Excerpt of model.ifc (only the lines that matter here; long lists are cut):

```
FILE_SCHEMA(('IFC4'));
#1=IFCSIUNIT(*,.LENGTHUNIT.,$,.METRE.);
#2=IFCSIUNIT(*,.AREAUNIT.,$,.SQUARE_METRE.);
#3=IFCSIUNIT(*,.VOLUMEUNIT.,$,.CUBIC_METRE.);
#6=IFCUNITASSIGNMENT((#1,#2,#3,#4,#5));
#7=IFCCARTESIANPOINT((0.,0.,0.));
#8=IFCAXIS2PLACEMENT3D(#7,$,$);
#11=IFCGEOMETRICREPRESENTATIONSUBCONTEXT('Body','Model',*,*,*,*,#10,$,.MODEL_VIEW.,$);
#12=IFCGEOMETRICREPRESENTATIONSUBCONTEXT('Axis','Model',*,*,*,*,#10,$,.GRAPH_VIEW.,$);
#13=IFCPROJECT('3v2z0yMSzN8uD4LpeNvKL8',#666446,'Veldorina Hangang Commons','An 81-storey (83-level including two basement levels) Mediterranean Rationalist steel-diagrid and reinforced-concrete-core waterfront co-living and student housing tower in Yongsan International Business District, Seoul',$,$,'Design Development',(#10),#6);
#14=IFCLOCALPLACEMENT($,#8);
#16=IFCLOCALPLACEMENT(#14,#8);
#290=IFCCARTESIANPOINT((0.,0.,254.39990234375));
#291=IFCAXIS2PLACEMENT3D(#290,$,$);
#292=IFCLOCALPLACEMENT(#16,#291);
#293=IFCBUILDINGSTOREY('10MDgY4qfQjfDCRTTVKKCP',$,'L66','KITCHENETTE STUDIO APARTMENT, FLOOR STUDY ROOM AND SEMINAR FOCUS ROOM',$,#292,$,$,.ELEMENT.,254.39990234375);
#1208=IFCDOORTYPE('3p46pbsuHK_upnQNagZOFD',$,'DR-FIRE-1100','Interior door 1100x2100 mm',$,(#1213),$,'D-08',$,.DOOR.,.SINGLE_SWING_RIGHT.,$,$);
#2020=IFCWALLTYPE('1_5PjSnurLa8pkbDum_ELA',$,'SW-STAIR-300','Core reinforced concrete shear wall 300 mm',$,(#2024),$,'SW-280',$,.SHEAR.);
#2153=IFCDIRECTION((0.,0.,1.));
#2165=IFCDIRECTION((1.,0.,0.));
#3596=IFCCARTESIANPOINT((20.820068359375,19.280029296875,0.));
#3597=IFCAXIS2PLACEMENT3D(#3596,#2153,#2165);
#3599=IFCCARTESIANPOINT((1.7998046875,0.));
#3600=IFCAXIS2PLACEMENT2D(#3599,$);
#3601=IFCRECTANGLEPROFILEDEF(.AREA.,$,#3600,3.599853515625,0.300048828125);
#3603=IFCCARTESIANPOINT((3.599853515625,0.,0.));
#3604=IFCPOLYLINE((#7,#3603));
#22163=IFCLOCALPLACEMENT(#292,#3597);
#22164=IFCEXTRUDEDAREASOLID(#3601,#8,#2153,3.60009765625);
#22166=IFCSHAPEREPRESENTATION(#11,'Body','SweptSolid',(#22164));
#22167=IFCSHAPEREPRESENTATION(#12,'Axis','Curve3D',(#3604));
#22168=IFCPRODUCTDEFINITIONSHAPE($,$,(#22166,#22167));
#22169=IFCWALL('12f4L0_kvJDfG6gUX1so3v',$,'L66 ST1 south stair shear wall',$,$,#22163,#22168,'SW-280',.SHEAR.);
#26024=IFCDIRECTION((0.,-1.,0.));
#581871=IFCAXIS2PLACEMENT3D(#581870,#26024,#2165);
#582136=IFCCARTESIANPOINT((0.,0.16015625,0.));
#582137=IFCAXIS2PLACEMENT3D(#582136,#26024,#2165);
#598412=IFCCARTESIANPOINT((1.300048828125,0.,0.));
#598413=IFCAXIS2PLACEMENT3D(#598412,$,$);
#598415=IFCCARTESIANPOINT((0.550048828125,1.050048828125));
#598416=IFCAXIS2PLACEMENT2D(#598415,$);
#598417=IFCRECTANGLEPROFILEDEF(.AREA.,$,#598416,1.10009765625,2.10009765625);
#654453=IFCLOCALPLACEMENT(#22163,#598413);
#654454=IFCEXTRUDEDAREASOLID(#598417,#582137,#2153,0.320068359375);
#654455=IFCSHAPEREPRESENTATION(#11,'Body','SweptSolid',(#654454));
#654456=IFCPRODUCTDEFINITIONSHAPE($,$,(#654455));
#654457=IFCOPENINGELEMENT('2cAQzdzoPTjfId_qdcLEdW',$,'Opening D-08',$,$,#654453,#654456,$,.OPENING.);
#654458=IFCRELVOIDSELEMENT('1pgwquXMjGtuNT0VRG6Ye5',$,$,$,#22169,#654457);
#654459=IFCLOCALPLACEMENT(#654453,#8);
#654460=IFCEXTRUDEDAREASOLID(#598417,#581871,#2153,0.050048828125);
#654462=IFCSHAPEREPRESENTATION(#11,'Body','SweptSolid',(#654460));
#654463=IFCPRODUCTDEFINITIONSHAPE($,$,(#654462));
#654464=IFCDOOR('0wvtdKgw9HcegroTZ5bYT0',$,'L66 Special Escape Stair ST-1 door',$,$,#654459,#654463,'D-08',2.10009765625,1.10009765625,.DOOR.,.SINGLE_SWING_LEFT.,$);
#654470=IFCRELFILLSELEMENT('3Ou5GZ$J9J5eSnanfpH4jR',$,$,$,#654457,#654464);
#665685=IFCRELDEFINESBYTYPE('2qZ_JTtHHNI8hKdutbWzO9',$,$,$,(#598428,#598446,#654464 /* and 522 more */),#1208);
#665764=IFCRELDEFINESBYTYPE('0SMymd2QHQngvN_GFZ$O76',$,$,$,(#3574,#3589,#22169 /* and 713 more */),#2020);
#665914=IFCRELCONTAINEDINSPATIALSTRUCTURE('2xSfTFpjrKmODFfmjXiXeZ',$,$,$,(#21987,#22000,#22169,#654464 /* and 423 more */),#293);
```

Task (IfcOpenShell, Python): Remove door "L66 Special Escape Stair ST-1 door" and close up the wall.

```python
import ifcopenshell
import ifcopenshell.api.feature
import ifcopenshell.api.root
import ifcopenshell.geom
import ifcopenshell.util.shape

model = ifcopenshell.open("model.ifc")
settings = ifcopenshell.geom.settings()


def volume(element):
    """Net volume in cubic metres, openings subtracted."""
    shape = ifcopenshell.geom.create_shape(settings, element)
    return ifcopenshell.util.shape.get_volume(shape.geometry)


door = model.by_guid("0wvtdKgw9HcegroTZ5bYT0")
opening = door.FillsVoids[0].RelatingOpeningElement
wall = opening.VoidsElements[0].RelatingBuildingElement
before = volume(wall)

ifcopenshell.api.root.remove_product(model, product=door)
ifcopenshell.api.feature.remove_feature(model, feature=opening)

after = volume(wall)

print(f"wall volume {before:.3f} -> {after:.3f} m3")

model.write("model_updated.ifc")
```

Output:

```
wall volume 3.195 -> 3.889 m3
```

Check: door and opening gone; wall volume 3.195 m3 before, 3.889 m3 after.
